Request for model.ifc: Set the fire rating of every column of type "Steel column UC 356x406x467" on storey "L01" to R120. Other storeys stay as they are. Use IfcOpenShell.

First a look at what the model holds.

```python
import ifcopenshell
import ifcopenshell.util.element

model = ifcopenshell.open("model.ifc")
print(model.schema)
storey = next(s for s in model.by_type("IfcBuildingStorey") if s.Name == "L01")
columns = [e for e in ifcopenshell.util.element.get_decomposition(storey) if e.is_a("IfcColumn")]
seen = {}
for e in columns:
    element_type = ifcopenshell.util.element.get_type(e)
    key = (element_type.Name if element_type != e and element_type else None, ifcopenshell.util.element.get_pset(e, "Pset_ColumnCommon", "FireRating"))
    seen[key] = seen.get(key, 0) + 1
for (name, value), count in sorted(seen.items(), key=str):
    print(count, "x", name, "|", value)
```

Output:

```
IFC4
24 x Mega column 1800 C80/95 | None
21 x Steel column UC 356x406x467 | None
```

```python
import ifcopenshell
import ifcopenshell.api.pset
import ifcopenshell.util.element

model = ifcopenshell.open("model.ifc")

storey = next(s for s in model.by_type("IfcBuildingStorey") if s.Name == "L01")
columns = [e for e in ifcopenshell.util.element.get_decomposition(storey) if e.is_a("IfcColumn")]

count = 0
for e in columns:
    element_type = ifcopenshell.util.element.get_type(e)
    if element_type in (None, e) or element_type.Name != "Steel column UC 356x406x467":
        continue
    found = ifcopenshell.util.element.get_pset(e, "Pset_ColumnCommon", should_inherit=False)
    if found:
        pset = model.by_id(found["id"])
        if len(ifcopenshell.util.element.get_elements_by_pset(pset)) > 1:
            pset = ifcopenshell.api.pset.unshare_pset(model, products=[e], pset=pset)[0]
    else:
        pset = ifcopenshell.api.pset.add_pset(model, product=e, name="Pset_ColumnCommon")
    ifcopenshell.api.pset.edit_pset(model, pset=pset, properties={"FireRating": "R120"})
    count += 1

print(count, "columns updated")

model.write("model_edited.ifc")
```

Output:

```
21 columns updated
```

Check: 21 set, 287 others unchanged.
